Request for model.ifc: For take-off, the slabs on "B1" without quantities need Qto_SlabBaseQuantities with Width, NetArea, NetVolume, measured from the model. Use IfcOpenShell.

First a look at what the model holds.

```python
import ifcopenshell
import ifcopenshell.util.element
import ifcopenshell.util.unit

model = ifcopenshell.open("model.ifc")
print(model.schema)
for unit_type in ("LENGTHUNIT", "AREAUNIT", "VOLUMEUNIT"):
    print(unit_type, ifcopenshell.util.unit.calculate_unit_scale(model, unit_type))
storey = next(s for s in model.by_type("IfcBuildingStorey") if s.Name == "B1")
slabs = [e for e in ifcopenshell.util.element.get_decomposition(storey) if e.is_a("IfcSlab")]
for e in sorted(slabs, key=lambda e: e.id()):
    print(e.id(), e.is_a(), e.Name, list(ifcopenshell.util.element.get_psets(e, qtos_only=True)), sep=" | ")
```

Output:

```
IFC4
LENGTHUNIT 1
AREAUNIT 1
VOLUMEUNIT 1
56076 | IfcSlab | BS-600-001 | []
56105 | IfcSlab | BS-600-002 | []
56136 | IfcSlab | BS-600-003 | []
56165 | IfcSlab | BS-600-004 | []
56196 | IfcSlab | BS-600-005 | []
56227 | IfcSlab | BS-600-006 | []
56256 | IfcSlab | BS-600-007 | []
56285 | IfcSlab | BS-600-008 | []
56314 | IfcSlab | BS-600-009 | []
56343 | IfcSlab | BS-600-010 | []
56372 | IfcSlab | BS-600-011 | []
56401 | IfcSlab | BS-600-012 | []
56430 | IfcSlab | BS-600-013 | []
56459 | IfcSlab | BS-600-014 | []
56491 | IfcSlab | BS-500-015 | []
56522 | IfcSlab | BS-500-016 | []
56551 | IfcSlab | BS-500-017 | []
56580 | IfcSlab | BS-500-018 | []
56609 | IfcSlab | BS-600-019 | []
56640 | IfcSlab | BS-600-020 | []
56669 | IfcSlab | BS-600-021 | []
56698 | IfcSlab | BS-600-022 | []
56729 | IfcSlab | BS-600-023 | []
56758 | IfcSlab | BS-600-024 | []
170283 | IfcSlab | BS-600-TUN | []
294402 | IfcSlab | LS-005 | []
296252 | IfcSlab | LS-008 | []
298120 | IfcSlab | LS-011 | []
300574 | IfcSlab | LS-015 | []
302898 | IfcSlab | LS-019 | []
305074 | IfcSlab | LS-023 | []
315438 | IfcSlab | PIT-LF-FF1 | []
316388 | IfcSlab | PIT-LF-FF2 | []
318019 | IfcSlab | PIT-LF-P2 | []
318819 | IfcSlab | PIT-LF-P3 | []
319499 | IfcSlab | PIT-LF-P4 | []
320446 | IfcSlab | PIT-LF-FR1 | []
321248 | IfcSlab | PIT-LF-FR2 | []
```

```python
import ifcopenshell
import ifcopenshell.api.pset
import ifcopenshell.geom
import ifcopenshell.util.element
import ifcopenshell.util.shape
import ifcopenshell.util.unit

model = ifcopenshell.open("model.ifc")
unit_scale = ifcopenshell.util.unit.calculate_unit_scale(model)
area_scale = ifcopenshell.util.unit.calculate_unit_scale(model, "AREAUNIT")
volume_scale = ifcopenshell.util.unit.calculate_unit_scale(model, "VOLUMEUNIT")
settings = ifcopenshell.geom.settings()

storey = next(s for s in model.by_type("IfcBuildingStorey") if s.Name == "B1")
slabs = [e for e in ifcopenshell.util.element.get_decomposition(storey) if e.is_a("IfcSlab")]

for e in sorted(slabs, key=lambda e: e.id()):
    if ifcopenshell.util.element.get_psets(e, qtos_only=True, should_inherit=False):
        continue
    # Geometry comes back in metres, in the element's own axes.
    shape = ifcopenshell.geom.create_shape(settings, e)
    values = {
        "Width": ifcopenshell.util.shape.get_z(shape.geometry) / unit_scale,
        "NetArea": ifcopenshell.util.shape.get_footprint_area(shape.geometry) / area_scale,
        "NetVolume": ifcopenshell.util.shape.get_volume(shape.geometry) / volume_scale,
    }
    qto = ifcopenshell.api.pset.add_qto(model, product=e, name="Qto_SlabBaseQuantities")
    ifcopenshell.api.pset.edit_qto(model, qto=qto, properties=values)
    print(e.id(), {k: round(v, 3) for k, v in values.items()})

model.write("model_edited.ifc")
```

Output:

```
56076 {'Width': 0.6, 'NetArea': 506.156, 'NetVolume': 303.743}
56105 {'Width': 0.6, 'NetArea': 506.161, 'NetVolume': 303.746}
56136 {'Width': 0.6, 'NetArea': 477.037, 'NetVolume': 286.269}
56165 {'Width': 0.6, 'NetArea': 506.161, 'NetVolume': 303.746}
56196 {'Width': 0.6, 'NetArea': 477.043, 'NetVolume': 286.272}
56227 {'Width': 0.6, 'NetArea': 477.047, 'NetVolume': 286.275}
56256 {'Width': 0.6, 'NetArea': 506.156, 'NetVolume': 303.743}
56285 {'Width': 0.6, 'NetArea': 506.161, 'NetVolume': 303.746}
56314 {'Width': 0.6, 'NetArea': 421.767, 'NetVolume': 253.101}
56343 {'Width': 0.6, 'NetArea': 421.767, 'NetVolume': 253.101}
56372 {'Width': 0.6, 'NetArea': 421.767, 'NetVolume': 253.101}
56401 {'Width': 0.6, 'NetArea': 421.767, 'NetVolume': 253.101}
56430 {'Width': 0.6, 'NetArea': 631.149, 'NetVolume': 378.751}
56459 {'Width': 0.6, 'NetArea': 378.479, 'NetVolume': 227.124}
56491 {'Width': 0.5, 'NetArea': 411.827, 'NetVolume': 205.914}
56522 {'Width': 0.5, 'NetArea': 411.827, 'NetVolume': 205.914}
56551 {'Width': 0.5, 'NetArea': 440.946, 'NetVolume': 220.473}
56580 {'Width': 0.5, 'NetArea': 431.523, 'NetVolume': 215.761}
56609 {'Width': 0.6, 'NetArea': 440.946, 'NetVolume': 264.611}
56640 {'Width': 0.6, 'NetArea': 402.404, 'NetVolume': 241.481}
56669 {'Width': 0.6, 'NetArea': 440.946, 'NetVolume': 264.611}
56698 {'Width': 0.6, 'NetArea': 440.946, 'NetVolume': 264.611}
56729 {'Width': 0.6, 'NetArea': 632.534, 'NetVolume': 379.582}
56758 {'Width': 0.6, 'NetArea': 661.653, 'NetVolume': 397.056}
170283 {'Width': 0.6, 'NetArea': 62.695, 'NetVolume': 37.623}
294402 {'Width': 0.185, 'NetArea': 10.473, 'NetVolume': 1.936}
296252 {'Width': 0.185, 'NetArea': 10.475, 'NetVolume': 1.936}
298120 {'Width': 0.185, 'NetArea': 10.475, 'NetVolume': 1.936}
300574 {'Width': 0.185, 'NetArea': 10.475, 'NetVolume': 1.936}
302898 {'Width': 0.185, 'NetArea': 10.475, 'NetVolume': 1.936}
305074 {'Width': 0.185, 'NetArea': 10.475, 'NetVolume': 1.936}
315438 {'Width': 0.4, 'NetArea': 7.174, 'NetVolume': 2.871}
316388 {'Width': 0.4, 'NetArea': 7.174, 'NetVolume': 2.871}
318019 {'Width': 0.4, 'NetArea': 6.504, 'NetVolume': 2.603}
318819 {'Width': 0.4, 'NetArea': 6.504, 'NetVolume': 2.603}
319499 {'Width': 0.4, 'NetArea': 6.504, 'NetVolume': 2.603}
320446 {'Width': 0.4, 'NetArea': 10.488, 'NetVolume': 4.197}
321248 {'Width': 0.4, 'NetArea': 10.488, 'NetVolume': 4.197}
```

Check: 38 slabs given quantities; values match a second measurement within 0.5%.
